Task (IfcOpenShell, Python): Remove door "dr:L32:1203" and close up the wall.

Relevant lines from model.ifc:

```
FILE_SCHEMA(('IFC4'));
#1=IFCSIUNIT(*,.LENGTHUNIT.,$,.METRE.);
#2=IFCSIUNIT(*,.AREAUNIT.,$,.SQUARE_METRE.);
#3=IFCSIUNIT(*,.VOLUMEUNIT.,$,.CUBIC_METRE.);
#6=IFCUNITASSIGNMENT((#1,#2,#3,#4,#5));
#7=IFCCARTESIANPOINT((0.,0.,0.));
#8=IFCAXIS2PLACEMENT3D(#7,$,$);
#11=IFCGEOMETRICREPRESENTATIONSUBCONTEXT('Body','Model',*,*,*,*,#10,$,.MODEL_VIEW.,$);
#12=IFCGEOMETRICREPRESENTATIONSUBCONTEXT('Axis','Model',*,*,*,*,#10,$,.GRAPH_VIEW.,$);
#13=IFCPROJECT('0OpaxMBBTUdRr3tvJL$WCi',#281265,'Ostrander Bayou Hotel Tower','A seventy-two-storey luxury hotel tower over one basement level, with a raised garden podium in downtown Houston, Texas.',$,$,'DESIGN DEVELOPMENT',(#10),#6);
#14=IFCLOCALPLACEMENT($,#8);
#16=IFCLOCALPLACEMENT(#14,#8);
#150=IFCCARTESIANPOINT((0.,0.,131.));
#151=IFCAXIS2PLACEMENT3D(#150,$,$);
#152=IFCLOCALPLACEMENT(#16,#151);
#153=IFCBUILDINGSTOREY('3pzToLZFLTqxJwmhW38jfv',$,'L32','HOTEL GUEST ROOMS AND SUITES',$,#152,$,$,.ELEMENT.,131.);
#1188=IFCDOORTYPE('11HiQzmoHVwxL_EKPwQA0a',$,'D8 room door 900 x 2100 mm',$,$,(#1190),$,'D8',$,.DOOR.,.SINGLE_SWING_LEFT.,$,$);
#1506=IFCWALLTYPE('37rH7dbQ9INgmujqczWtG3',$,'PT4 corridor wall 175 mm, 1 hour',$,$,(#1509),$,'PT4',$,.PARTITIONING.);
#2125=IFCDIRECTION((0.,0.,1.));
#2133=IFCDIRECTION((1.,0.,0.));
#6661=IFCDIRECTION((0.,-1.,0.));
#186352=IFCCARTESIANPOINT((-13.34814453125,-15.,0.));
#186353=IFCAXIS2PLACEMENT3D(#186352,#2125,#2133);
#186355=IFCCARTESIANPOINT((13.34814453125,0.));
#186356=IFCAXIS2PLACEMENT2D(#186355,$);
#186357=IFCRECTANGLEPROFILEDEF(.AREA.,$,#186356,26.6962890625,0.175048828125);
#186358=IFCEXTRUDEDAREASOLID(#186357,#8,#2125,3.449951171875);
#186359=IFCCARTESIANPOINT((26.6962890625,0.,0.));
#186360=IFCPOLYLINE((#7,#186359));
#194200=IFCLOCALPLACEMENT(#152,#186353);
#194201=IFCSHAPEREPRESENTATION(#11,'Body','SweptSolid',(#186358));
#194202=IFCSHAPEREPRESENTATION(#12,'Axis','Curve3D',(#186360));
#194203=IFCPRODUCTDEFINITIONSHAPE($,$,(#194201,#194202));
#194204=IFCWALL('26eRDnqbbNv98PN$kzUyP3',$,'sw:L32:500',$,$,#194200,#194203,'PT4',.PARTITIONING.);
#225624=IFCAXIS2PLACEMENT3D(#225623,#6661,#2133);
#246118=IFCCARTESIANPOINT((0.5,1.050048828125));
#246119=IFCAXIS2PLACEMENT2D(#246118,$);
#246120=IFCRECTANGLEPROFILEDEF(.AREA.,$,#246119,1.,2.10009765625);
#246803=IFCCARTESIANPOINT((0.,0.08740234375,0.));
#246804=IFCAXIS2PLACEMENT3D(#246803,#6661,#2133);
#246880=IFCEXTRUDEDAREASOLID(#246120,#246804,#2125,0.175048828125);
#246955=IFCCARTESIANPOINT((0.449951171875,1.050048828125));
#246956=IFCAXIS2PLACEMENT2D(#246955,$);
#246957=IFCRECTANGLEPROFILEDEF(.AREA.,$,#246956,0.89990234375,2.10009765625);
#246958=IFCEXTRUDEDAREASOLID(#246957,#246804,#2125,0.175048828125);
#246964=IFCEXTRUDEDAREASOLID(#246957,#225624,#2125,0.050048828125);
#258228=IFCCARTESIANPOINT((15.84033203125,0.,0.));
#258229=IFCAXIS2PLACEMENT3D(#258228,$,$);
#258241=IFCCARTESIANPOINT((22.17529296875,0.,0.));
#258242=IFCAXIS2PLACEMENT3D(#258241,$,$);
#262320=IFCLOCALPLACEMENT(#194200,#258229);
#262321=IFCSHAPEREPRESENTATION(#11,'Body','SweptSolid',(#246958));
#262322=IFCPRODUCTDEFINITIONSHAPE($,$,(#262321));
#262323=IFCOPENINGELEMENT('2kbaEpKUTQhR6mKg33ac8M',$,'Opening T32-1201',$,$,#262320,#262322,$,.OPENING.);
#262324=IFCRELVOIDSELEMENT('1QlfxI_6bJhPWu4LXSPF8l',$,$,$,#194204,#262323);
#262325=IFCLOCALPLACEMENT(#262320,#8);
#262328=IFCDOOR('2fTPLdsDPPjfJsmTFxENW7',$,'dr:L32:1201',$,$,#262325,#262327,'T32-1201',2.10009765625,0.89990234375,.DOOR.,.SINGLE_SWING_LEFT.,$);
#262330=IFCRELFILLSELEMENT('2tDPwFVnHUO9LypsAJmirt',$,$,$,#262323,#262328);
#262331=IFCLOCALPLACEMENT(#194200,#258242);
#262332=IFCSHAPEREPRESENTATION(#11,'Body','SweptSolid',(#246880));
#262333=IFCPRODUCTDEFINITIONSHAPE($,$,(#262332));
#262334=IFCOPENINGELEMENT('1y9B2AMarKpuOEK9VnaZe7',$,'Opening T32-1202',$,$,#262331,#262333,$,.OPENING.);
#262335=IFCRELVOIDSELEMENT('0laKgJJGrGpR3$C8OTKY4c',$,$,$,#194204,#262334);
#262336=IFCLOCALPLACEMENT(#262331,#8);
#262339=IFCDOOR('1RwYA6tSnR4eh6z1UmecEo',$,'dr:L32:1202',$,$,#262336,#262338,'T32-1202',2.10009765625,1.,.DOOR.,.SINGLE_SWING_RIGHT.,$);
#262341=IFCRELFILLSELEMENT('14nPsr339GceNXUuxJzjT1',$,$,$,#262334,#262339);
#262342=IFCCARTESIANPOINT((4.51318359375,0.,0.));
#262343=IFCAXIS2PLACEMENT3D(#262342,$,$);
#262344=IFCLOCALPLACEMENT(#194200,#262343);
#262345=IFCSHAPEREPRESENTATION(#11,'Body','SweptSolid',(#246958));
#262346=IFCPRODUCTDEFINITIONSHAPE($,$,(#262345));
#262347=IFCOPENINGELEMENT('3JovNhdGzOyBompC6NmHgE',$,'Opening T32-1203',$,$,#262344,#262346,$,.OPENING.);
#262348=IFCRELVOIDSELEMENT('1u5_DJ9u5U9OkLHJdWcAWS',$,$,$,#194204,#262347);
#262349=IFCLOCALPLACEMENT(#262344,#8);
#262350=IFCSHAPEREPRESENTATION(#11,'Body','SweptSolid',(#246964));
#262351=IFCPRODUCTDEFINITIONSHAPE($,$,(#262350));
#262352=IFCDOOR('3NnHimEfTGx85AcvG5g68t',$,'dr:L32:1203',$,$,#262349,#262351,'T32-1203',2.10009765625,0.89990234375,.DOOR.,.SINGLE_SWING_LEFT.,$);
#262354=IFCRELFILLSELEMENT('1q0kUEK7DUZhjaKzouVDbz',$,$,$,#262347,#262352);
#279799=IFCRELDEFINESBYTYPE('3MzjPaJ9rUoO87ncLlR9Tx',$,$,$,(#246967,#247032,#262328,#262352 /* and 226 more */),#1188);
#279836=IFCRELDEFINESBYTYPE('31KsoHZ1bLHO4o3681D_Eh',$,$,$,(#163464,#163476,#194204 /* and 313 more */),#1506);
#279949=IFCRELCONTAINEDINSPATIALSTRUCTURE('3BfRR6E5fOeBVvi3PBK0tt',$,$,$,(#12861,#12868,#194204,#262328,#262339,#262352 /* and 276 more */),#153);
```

```python
import ifcopenshell
import ifcopenshell.api.feature
import ifcopenshell.api.root
import ifcopenshell.geom
import ifcopenshell.util.shape

model = ifcopenshell.open("model.ifc")
settings = ifcopenshell.geom.settings()


def volume(element):
    """Net volume in cubic metres, openings subtracted."""
    shape = ifcopenshell.geom.create_shape(settings, element)
    return ifcopenshell.util.shape.get_volume(shape.geometry)


door = model.by_guid("3NnHimEfTGx85AcvG5g68t")
opening = door.FillsVoids[0].RelatingOpeningElement
wall = opening.VoidsElements[0].RelatingBuildingElement
before = volume(wall)

ifcopenshell.api.root.remove_product(model, product=door)
ifcopenshell.api.feature.remove_feature(model, feature=opening)

after = volume(wall)

print(f"wall volume {before:.3f} -> {after:.3f} m3")

model.write("model_updated.ifc")
```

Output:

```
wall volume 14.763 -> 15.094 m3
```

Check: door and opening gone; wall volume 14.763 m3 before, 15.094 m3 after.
